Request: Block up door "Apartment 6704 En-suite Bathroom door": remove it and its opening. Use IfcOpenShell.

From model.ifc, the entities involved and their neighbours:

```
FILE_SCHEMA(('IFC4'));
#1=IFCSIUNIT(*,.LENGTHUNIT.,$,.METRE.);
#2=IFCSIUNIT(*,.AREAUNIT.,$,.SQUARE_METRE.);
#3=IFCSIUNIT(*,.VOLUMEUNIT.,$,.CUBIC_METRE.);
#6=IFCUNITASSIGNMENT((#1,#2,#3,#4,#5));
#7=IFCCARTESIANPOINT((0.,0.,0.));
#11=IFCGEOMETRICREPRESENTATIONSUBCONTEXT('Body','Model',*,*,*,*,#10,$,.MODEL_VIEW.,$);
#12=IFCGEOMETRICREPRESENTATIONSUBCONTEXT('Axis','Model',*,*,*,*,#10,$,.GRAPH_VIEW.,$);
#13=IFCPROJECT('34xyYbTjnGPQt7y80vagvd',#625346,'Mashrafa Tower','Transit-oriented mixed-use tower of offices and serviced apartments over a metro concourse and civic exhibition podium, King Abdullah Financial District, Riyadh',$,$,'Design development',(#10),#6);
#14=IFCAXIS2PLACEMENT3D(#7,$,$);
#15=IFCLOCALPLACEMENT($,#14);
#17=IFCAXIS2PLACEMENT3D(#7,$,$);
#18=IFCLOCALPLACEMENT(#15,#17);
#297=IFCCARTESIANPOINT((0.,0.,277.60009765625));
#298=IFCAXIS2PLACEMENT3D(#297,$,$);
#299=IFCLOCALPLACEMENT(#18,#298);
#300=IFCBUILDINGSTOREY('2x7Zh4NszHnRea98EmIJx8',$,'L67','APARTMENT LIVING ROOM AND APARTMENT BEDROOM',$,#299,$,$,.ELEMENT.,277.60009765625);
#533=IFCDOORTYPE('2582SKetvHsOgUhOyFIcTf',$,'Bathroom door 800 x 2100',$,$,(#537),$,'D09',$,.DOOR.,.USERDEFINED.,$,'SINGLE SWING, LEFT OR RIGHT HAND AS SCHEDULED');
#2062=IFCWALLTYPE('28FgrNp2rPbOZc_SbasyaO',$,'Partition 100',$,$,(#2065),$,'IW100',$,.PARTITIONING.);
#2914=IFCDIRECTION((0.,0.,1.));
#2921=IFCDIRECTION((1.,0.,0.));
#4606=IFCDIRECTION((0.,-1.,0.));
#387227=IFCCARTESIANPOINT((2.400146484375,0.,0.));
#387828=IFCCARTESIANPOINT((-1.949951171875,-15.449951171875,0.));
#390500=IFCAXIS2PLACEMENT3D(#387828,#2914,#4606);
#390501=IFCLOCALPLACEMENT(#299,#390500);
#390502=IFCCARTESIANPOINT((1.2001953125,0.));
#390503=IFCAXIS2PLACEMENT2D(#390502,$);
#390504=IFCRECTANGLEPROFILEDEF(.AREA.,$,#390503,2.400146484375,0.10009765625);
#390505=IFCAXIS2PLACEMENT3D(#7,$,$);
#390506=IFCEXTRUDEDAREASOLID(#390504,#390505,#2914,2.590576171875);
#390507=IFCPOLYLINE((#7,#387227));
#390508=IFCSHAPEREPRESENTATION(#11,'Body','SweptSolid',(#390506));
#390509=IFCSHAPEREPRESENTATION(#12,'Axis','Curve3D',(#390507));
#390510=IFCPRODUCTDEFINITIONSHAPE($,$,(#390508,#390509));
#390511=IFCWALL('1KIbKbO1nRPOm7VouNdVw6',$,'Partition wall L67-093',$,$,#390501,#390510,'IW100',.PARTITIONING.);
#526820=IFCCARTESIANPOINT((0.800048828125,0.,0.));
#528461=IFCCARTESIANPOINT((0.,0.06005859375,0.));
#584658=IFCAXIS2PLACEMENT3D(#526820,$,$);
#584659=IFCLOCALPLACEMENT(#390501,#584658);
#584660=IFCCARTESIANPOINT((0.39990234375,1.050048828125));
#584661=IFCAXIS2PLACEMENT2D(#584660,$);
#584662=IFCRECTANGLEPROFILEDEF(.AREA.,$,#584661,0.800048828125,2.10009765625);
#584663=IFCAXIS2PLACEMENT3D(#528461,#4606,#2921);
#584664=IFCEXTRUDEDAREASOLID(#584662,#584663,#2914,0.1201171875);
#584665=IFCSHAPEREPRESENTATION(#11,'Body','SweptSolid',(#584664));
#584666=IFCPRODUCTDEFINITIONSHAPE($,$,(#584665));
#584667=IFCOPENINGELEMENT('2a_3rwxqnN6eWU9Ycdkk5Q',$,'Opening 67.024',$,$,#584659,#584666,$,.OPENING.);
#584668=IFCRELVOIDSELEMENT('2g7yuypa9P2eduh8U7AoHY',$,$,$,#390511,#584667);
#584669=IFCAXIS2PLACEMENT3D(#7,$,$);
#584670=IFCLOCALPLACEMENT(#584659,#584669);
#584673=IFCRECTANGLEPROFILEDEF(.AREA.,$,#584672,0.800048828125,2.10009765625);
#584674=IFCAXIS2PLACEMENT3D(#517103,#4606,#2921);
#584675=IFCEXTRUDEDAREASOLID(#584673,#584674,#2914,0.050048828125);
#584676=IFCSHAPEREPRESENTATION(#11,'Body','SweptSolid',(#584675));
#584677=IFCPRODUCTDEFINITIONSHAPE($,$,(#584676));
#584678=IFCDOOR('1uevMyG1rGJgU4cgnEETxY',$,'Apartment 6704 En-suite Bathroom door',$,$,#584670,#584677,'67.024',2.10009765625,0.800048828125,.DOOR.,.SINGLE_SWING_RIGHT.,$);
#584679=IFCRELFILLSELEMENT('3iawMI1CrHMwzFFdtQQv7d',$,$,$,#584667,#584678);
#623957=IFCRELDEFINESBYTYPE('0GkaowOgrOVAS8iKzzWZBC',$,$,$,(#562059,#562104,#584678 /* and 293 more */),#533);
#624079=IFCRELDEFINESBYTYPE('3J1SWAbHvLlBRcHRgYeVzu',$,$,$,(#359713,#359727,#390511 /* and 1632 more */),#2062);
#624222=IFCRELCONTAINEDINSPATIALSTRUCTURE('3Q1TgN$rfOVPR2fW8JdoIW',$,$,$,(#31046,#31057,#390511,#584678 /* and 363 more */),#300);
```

```python
import ifcopenshell
import ifcopenshell.api.feature
import ifcopenshell.api.root
import ifcopenshell.geom
import ifcopenshell.util.shape

model = ifcopenshell.open("model.ifc")
settings = ifcopenshell.geom.settings()


def volume(element):
    """Net volume in cubic metres, openings subtracted."""
    shape = ifcopenshell.geom.create_shape(settings, element)
    return ifcopenshell.util.shape.get_volume(shape.geometry)


door = model.by_guid("1uevMyG1rGJgU4cgnEETxY")
opening = door.FillsVoids[0].RelatingOpeningElement
wall = opening.VoidsElements[0].RelatingBuildingElement
before = volume(wall)

ifcopenshell.api.root.remove_product(model, product=door)
ifcopenshell.api.feature.remove_feature(model, feature=opening)

after = volume(wall)

print(f"wall volume {before:.3f} -> {after:.3f} m3")

model.write("model_v2.ifc")
```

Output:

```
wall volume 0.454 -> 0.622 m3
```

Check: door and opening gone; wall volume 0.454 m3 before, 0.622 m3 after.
